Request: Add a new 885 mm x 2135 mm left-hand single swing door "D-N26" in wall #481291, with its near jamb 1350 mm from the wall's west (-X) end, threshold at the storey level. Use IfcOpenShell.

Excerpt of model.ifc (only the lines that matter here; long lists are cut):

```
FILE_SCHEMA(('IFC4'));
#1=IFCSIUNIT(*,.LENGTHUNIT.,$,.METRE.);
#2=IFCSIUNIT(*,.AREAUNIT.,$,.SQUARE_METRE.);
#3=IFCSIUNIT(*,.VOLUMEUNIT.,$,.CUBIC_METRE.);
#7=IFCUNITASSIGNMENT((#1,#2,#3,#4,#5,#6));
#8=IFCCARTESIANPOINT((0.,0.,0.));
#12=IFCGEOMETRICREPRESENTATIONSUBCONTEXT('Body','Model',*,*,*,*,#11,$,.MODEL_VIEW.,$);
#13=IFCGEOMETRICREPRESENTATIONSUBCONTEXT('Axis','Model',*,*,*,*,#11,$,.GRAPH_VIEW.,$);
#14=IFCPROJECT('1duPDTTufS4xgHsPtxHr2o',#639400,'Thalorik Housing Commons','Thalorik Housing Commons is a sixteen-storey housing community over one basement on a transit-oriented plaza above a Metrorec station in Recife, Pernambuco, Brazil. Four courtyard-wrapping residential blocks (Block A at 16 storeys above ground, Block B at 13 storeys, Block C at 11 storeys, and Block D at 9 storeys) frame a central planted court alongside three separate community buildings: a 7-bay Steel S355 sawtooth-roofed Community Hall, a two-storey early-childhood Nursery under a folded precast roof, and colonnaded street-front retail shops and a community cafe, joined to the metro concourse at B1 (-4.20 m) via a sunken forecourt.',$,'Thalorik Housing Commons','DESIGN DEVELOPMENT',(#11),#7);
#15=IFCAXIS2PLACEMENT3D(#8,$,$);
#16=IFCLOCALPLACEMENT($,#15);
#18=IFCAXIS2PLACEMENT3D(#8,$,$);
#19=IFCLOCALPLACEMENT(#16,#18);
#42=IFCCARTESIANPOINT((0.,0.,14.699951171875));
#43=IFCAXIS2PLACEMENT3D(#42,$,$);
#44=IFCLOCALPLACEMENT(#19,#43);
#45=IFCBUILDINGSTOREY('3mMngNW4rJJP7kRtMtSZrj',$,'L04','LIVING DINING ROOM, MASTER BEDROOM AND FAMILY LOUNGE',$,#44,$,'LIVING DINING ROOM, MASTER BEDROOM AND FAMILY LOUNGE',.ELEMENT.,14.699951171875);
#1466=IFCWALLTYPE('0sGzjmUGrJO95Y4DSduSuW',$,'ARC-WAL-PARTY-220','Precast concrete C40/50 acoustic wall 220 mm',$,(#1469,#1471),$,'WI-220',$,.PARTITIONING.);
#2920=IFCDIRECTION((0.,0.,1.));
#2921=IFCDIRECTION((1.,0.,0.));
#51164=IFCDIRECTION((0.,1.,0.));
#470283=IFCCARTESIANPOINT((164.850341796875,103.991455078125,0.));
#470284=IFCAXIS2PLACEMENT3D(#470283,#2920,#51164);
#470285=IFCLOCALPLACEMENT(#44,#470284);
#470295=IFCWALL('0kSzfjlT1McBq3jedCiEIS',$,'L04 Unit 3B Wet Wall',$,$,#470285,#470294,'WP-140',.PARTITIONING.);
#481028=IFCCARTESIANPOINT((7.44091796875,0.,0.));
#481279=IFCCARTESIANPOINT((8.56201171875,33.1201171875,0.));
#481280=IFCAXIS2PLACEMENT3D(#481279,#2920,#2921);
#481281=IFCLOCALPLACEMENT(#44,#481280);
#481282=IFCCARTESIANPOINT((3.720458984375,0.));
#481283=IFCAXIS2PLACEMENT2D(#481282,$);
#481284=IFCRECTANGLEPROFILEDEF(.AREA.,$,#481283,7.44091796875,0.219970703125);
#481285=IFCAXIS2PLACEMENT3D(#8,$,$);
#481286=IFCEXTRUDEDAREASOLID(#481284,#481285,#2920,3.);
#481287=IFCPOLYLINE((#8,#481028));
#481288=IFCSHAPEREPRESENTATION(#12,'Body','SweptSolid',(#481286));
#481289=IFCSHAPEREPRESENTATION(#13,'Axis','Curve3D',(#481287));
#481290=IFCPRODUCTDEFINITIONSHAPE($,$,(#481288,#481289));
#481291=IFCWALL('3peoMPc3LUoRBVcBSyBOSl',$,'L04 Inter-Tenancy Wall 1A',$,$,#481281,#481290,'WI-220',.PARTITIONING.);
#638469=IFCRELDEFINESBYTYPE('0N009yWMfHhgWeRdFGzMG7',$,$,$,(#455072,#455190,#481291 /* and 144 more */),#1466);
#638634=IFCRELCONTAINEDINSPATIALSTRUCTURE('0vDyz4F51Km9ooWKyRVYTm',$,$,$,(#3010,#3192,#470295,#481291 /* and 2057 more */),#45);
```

```python
import numpy as np
import ifcopenshell
import ifcopenshell.api.feature
import ifcopenshell.api.geometry
import ifcopenshell.api.root
import ifcopenshell.api.spatial
import ifcopenshell.geom
import ifcopenshell.util.element
import ifcopenshell.util.placement
import ifcopenshell.util.representation
import ifcopenshell.util.shape
import ifcopenshell.util.unit

model = ifcopenshell.open("model.ifc")
unit_scale = ifcopenshell.util.unit.calculate_unit_scale(model)
settings = ifcopenshell.geom.settings()


def volume(element):
    """Net volume in cubic metres, openings subtracted."""
    shape = ifcopenshell.geom.create_shape(settings, element)
    return ifcopenshell.util.shape.get_volume(shape.geometry)


wall = model.by_id(481291)
storey = ifcopenshell.util.element.get_container(wall, ifc_class="IfcBuildingStorey")
context = ifcopenshell.util.representation.get_context(model, "Model", "Body", "MODEL_VIEW")
before = volume(wall)

width, height, from_end, sill = 0.885, 2.135, 1.35, 0.0  # metres

# The wall runs along its own X axis, and the end named is its -X end.
wall_shape = ifcopenshell.geom.create_shape(settings, wall)
x, y, z = ifcopenshell.util.shape.get_vertices(wall_shape.geometry).T
start = x.min() + from_end
face, thickness = float(y.min()), float(y.max() - y.min())
wall_matrix = ifcopenshell.util.placement.get_local_placement(wall.ObjectPlacement)
level = ifcopenshell.util.placement.get_local_placement(storey.ObjectPlacement)[2, 3]


def in_wall(x, y):
    """Placement at x, y metres in the wall's axes, at sill height."""
    matrix = wall_matrix.copy()
    matrix[:, 3] = wall_matrix @ np.array([x / unit_scale, y / unit_scale, 0.0, 1.0])
    matrix[2, 3] = level + sill / unit_scale
    return matrix


# Opening: a box that overshoots both wall faces by 50 mm.
opening = ifcopenshell.api.root.create_entity(model, ifc_class="IfcOpeningElement", predefined_type="OPENING")
box = ifcopenshell.api.geometry.add_wall_representation(
    model, context=context, length=width, height=height, thickness=thickness + 0.1
)
ifcopenshell.api.geometry.assign_representation(model, product=opening, representation=box)
ifcopenshell.api.geometry.edit_object_placement(model, product=opening, matrix=in_wall(start, face - 0.05), is_si=False)
ifcopenshell.api.feature.add_feature(model, feature=opening, element=wall)

door = ifcopenshell.api.root.create_entity(model, ifc_class="IfcDoor", name="D-N26", predefined_type="DOOR")
door.OverallWidth, door.OverallHeight = width / unit_scale, height / unit_scale
door.OperationType = "SINGLE_SWING_LEFT"
body = ifcopenshell.api.geometry.add_door_representation(
    model,
    context=context,
    overall_width=door.OverallWidth,
    overall_height=door.OverallHeight,
    operation_type="SINGLE_SWING_LEFT",
    lining_properties={"LiningDepth": thickness / unit_scale, "ThresholdDepth": thickness / unit_scale},
)
ifcopenshell.api.geometry.assign_representation(model, product=door, representation=body)
ifcopenshell.api.spatial.assign_container(model, products=[door], relating_structure=storey)
ifcopenshell.api.feature.add_filling(model, opening=opening, element=door)

# The lining spans the wall, so the door starts at the wall face.
ifcopenshell.api.geometry.edit_object_placement(model, product=door, matrix=in_wall(start, face), is_si=False)

after = volume(wall)

print(f"wall volume {before:.3f} -> {after:.3f} m3")

model.write("model_edited.ifc")
```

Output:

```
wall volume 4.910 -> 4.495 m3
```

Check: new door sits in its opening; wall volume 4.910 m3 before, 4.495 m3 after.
